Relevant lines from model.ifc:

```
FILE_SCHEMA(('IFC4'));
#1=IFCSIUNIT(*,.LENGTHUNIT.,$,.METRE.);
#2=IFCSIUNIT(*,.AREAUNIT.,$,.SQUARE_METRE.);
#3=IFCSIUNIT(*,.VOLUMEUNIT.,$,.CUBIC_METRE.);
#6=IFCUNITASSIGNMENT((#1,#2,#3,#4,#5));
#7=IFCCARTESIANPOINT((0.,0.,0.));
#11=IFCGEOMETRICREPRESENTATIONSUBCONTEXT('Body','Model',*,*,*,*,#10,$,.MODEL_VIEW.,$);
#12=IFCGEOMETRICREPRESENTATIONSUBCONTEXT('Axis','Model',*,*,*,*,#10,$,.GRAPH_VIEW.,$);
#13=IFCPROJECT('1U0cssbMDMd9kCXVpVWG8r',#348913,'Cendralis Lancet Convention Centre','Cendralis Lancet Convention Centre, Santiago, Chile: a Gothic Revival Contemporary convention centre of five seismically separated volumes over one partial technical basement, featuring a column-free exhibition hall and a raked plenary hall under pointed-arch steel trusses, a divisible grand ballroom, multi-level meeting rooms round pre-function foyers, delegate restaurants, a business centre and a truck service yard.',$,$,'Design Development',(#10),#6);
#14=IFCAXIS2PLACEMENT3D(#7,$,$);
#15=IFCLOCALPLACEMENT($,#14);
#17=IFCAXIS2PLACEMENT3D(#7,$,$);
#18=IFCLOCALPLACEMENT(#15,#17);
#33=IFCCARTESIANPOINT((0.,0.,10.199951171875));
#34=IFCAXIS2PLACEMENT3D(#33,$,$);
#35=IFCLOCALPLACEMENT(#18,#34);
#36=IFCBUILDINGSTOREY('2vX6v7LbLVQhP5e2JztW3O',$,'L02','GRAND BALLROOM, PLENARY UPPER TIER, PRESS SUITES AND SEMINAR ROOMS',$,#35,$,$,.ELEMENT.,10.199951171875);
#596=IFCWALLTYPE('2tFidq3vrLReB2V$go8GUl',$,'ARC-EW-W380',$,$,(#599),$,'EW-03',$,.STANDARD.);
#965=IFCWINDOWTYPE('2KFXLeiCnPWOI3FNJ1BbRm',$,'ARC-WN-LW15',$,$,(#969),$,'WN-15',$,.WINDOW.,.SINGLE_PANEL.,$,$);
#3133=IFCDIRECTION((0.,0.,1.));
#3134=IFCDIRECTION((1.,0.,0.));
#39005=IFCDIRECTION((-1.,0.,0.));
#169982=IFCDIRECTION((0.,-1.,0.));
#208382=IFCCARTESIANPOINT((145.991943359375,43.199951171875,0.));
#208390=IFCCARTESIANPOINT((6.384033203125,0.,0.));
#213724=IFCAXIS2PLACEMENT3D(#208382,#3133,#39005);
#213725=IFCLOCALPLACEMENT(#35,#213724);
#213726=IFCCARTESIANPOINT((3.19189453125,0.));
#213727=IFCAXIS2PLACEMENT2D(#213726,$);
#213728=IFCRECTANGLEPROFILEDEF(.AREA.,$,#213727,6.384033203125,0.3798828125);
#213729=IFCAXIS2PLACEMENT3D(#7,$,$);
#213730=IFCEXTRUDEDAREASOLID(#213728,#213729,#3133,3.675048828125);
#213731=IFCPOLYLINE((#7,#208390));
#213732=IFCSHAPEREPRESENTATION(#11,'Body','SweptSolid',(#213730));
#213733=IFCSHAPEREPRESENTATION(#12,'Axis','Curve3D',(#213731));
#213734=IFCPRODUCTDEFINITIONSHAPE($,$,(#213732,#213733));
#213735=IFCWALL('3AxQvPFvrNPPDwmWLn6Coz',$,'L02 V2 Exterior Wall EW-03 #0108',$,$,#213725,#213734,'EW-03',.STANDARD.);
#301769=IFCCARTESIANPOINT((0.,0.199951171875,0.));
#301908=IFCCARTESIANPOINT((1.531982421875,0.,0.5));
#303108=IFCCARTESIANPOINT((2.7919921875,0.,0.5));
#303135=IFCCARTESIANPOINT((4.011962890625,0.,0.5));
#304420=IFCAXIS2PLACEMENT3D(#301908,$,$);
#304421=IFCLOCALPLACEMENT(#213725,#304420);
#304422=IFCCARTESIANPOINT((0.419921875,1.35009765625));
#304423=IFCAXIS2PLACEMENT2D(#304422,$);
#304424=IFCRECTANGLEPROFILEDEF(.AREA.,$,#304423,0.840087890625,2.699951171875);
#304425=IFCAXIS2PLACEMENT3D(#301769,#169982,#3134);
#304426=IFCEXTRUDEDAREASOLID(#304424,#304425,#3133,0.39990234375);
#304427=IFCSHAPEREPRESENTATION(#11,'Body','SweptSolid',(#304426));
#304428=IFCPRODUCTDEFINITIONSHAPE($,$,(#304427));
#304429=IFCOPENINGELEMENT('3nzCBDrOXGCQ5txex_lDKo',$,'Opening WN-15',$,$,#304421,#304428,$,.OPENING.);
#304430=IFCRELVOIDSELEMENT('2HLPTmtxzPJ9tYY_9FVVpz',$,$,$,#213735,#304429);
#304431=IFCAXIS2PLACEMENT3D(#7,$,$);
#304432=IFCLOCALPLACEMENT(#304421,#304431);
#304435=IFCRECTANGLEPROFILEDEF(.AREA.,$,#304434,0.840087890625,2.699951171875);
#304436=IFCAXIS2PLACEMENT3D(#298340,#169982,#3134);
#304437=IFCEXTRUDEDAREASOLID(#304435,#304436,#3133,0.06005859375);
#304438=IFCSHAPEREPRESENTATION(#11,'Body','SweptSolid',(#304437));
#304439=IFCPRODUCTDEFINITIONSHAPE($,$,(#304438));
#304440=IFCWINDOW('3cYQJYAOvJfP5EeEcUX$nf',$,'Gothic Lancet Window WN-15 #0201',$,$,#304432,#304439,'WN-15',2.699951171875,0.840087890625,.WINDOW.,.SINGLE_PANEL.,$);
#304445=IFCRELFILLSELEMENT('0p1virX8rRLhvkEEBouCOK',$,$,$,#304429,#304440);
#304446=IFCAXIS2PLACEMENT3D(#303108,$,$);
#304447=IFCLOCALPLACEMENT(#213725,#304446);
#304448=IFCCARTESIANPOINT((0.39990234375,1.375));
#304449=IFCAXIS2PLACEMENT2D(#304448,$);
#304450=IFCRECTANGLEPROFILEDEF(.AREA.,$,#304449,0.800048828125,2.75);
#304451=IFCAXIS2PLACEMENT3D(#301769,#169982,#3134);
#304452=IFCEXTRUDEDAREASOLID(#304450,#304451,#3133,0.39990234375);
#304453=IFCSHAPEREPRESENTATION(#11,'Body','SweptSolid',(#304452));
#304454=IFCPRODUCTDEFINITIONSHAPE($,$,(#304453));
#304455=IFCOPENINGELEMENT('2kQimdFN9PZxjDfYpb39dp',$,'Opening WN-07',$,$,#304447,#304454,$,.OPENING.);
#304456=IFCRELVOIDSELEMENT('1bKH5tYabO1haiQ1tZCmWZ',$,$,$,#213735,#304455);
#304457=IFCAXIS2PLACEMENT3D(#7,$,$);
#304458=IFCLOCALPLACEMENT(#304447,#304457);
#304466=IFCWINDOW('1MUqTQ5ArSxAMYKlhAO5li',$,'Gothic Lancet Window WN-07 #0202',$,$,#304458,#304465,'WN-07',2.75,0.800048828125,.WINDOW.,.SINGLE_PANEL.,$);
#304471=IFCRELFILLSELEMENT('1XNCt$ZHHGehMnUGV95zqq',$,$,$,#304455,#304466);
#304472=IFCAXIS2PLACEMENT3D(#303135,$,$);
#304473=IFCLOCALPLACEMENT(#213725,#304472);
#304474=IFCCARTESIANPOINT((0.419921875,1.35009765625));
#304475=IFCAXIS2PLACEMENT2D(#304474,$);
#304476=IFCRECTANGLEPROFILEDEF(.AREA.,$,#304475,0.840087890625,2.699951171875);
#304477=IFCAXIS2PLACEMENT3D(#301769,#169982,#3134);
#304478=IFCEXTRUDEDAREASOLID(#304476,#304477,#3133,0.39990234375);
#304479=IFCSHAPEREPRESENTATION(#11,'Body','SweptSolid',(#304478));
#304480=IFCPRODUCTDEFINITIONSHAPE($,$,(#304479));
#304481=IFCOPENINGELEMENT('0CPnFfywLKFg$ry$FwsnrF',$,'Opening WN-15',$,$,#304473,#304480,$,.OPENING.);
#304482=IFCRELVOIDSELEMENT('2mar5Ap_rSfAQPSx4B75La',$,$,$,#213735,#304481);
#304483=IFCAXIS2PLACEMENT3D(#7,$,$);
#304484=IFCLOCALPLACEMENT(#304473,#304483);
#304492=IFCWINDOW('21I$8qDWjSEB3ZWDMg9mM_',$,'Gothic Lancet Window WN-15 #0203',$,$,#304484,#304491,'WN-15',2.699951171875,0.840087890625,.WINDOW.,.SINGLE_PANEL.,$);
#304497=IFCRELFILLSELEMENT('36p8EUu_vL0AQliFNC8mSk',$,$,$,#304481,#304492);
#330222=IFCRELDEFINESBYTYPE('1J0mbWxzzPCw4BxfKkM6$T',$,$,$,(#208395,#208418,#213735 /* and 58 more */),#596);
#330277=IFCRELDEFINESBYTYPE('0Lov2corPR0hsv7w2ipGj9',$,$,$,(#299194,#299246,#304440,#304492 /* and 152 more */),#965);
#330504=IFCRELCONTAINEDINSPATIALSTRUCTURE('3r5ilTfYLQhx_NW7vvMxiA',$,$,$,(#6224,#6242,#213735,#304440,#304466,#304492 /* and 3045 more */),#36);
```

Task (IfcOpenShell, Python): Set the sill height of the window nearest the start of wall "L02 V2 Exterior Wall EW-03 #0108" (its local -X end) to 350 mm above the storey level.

```python
import numpy as np
import ifcopenshell
import ifcopenshell.api.geometry
import ifcopenshell.geom
import ifcopenshell.util.element
import ifcopenshell.util.placement
import ifcopenshell.util.shape
import ifcopenshell.util.unit

model = ifcopenshell.open("model.ifc")
unit_scale = ifcopenshell.util.unit.calculate_unit_scale(model)

window = model.by_guid("3cYQJYAOvJfP5EeEcUX$nf")
opening = window.FillsVoids[0].RelatingOpeningElement
storey = ifcopenshell.util.element.get_container(window, ifc_class="IfcBuildingStorey")
level = ifcopenshell.util.placement.get_local_placement(storey.ObjectPlacement)[2, 3]

# The opening's origin need not be at the sill, so measure its lowest point.
shape = ifcopenshell.geom.create_shape(ifcopenshell.geom.settings(), opening)
bottom = ifcopenshell.util.shape.get_shape_bottom_elevation(shape, shape.geometry) / unit_scale
dz = level + 0.35 - bottom

shift = np.array([0.0, 0.0, dz])
# The window is placed relative to its opening, so it follows when the opening moves.
matrix = ifcopenshell.util.placement.get_local_placement(opening.ObjectPlacement)
matrix[:3, 3] += shift
ifcopenshell.api.geometry.edit_object_placement(
    model, product=opening, matrix=matrix, is_si=False, should_transform_children=True
)

print(f"moved by {dz * unit_scale:+.3f} m")

model.write("model_v2.ifc")
```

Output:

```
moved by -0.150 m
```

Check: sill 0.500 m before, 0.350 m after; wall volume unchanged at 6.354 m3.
